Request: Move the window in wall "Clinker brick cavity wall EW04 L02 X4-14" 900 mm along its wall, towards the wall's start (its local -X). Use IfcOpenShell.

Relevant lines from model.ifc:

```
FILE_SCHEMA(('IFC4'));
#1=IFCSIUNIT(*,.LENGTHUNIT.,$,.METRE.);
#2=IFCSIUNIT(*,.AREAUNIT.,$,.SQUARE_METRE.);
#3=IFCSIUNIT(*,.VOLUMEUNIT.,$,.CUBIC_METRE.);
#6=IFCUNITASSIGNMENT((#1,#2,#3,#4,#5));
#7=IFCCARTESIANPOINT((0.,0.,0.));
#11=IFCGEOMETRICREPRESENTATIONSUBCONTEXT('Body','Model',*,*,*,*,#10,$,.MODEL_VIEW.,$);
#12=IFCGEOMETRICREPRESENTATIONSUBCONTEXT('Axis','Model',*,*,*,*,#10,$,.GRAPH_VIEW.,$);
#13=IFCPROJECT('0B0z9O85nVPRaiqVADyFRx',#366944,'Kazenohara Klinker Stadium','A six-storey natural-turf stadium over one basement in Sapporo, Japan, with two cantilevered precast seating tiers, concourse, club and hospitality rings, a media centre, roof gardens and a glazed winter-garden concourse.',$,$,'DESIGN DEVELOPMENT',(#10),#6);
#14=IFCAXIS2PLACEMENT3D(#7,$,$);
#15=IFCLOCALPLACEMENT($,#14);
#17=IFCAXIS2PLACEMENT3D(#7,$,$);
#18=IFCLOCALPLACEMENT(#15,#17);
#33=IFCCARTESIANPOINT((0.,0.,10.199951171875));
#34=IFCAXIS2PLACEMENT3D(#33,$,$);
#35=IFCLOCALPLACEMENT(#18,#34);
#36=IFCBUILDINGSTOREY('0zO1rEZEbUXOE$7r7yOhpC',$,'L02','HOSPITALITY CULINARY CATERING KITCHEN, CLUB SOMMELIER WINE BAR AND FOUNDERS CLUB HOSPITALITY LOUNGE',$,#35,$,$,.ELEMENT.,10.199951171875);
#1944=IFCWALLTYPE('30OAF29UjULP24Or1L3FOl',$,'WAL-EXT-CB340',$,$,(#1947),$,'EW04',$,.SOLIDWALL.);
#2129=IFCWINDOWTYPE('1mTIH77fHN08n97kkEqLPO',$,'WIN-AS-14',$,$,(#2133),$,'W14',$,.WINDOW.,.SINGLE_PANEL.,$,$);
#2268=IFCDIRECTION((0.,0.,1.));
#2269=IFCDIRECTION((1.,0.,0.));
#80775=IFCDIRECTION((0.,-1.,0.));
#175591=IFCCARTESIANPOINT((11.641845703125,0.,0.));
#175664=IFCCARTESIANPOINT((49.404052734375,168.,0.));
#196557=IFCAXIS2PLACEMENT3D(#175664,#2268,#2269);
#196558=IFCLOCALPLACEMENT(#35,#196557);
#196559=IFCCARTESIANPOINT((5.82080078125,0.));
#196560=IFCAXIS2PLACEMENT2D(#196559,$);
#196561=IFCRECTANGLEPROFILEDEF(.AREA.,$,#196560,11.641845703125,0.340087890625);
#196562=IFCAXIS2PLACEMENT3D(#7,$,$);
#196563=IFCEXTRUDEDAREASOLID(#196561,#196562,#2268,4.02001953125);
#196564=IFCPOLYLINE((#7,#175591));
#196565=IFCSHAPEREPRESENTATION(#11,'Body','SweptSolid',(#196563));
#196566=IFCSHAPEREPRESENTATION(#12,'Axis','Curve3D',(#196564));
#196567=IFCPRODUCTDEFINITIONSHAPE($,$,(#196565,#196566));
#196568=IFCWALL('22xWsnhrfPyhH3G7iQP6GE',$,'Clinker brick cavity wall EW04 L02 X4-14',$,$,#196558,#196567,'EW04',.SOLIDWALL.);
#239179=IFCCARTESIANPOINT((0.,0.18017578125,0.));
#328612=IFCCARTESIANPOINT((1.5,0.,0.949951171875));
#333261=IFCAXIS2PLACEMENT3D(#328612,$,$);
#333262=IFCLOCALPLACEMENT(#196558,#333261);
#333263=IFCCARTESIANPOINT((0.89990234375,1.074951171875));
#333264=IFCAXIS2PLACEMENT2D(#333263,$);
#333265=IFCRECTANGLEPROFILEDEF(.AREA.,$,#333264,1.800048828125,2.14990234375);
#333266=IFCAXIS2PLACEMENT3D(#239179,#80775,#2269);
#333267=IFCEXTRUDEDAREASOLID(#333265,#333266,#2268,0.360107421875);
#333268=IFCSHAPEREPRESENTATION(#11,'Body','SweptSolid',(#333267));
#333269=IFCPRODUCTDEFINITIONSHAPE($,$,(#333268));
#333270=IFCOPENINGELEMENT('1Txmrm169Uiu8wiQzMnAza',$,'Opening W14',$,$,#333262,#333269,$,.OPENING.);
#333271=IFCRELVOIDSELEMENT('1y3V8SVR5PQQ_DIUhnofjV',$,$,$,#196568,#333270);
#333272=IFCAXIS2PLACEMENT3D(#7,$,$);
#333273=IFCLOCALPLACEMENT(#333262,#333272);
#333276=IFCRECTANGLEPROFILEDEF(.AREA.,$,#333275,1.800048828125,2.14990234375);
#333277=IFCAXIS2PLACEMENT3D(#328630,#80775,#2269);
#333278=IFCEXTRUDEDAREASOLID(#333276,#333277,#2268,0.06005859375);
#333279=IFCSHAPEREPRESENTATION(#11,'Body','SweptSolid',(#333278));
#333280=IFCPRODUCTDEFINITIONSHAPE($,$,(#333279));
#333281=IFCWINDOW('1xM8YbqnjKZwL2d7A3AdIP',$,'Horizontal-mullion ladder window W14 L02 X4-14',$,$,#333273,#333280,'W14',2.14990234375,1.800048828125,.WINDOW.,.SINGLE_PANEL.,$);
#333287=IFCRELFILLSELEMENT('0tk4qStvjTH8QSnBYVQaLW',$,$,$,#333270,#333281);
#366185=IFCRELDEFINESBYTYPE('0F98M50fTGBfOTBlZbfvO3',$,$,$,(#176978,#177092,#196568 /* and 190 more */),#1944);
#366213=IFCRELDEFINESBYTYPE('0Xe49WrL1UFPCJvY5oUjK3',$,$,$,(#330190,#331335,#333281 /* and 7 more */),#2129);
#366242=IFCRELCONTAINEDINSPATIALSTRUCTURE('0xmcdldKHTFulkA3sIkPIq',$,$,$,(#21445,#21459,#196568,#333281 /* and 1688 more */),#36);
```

```python
import ifcopenshell
import ifcopenshell.api.geometry
import ifcopenshell.util.placement

model = ifcopenshell.open("model.ifc")

window = model.by_id(333281)
opening = window.FillsVoids[0].RelatingOpeningElement
wall = opening.VoidsElements[0].RelatingBuildingElement

wall_matrix = ifcopenshell.util.placement.get_local_placement(wall.ObjectPlacement)
shift = wall_matrix[:3, 0] * -0.9
before = ifcopenshell.util.placement.get_local_placement(window.ObjectPlacement)[:3, 3].copy()

# The window is placed relative to its opening, so it follows when the opening moves.
matrix = ifcopenshell.util.placement.get_local_placement(opening.ObjectPlacement)
matrix[:3, 3] += shift
ifcopenshell.api.geometry.edit_object_placement(
    model, product=opening, matrix=matrix, is_si=False, should_transform_children=True
)

after = ifcopenshell.util.placement.get_local_placement(window.ObjectPlacement)[:3, 3]
print("window moved by", (after - before).round(3) + 0.0)

model.write("model_rev.ifc")
```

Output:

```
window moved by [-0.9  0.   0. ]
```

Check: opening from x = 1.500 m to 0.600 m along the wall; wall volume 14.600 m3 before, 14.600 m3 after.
